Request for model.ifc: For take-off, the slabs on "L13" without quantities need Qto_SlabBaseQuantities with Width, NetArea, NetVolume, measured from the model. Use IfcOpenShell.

First a look at what the model holds.

```python
import ifcopenshell
import ifcopenshell.util.element
import ifcopenshell.util.unit

model = ifcopenshell.open("model.ifc")
print(model.schema)
for unit_type in ("LENGTHUNIT", "AREAUNIT", "VOLUMEUNIT"):
    print(unit_type, ifcopenshell.util.unit.calculate_unit_scale(model, unit_type))
storey = next(s for s in model.by_type("IfcBuildingStorey") if s.Name == "L13")
slabs = [e for e in ifcopenshell.util.element.get_decomposition(storey) if e.is_a("IfcSlab")]
for e in sorted(slabs, key=lambda e: e.id()):
    print(e.id(), e.is_a(), e.Name, list(ifcopenshell.util.element.get_psets(e, qtos_only=True)), sep=" | ")
```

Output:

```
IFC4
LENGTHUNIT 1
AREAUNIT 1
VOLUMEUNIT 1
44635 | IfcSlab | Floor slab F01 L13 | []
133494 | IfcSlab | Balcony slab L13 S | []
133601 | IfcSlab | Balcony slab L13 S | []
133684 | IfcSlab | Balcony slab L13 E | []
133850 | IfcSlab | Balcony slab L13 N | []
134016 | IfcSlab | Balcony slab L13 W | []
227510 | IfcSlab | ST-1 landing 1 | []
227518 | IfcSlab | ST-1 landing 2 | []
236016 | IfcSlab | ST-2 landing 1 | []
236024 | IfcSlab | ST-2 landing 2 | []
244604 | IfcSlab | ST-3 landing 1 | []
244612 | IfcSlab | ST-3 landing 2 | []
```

```python
import ifcopenshell
import ifcopenshell.api.pset
import ifcopenshell.geom
import ifcopenshell.util.element
import ifcopenshell.util.shape
import ifcopenshell.util.unit

model = ifcopenshell.open("model.ifc")
unit_scale = ifcopenshell.util.unit.calculate_unit_scale(model)
area_scale = ifcopenshell.util.unit.calculate_unit_scale(model, "AREAUNIT")
volume_scale = ifcopenshell.util.unit.calculate_unit_scale(model, "VOLUMEUNIT")
settings = ifcopenshell.geom.settings()

storey = next(s for s in model.by_type("IfcBuildingStorey") if s.Name == "L13")
slabs = [e for e in ifcopenshell.util.element.get_decomposition(storey) if e.is_a("IfcSlab")]

for e in sorted(slabs, key=lambda e: e.id()):
    if ifcopenshell.util.element.get_psets(e, qtos_only=True, should_inherit=False):
        continue
    # Geometry comes back in metres, in the element's own axes.
    shape = ifcopenshell.geom.create_shape(settings, e)
    values = {
        "Width": ifcopenshell.util.shape.get_z(shape.geometry) / unit_scale,
        "NetArea": ifcopenshell.util.shape.get_footprint_area(shape.geometry) / area_scale,
        "NetVolume": ifcopenshell.util.shape.get_volume(shape.geometry) / volume_scale,
    }
    qto = ifcopenshell.api.pset.add_qto(model, product=e, name="Qto_SlabBaseQuantities")
    ifcopenshell.api.pset.edit_qto(model, qto=qto, properties=values)
    print(e.id(), {k: round(v, 3) for k, v in values.items()})

model.write("model-out.ifc")
```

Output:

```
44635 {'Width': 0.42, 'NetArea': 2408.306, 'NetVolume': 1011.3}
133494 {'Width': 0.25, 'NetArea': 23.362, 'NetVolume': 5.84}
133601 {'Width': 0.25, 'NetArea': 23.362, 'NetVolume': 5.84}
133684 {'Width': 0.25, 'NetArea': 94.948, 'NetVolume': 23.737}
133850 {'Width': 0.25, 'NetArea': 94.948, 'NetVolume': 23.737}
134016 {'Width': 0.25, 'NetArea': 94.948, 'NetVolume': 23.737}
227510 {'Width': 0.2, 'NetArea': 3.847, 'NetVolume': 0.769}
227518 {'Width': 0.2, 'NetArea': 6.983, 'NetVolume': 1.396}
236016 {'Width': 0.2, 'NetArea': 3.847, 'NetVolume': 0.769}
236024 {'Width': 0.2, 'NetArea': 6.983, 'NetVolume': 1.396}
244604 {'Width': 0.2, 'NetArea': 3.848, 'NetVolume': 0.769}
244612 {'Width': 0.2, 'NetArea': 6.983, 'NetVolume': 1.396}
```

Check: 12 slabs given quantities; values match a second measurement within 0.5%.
